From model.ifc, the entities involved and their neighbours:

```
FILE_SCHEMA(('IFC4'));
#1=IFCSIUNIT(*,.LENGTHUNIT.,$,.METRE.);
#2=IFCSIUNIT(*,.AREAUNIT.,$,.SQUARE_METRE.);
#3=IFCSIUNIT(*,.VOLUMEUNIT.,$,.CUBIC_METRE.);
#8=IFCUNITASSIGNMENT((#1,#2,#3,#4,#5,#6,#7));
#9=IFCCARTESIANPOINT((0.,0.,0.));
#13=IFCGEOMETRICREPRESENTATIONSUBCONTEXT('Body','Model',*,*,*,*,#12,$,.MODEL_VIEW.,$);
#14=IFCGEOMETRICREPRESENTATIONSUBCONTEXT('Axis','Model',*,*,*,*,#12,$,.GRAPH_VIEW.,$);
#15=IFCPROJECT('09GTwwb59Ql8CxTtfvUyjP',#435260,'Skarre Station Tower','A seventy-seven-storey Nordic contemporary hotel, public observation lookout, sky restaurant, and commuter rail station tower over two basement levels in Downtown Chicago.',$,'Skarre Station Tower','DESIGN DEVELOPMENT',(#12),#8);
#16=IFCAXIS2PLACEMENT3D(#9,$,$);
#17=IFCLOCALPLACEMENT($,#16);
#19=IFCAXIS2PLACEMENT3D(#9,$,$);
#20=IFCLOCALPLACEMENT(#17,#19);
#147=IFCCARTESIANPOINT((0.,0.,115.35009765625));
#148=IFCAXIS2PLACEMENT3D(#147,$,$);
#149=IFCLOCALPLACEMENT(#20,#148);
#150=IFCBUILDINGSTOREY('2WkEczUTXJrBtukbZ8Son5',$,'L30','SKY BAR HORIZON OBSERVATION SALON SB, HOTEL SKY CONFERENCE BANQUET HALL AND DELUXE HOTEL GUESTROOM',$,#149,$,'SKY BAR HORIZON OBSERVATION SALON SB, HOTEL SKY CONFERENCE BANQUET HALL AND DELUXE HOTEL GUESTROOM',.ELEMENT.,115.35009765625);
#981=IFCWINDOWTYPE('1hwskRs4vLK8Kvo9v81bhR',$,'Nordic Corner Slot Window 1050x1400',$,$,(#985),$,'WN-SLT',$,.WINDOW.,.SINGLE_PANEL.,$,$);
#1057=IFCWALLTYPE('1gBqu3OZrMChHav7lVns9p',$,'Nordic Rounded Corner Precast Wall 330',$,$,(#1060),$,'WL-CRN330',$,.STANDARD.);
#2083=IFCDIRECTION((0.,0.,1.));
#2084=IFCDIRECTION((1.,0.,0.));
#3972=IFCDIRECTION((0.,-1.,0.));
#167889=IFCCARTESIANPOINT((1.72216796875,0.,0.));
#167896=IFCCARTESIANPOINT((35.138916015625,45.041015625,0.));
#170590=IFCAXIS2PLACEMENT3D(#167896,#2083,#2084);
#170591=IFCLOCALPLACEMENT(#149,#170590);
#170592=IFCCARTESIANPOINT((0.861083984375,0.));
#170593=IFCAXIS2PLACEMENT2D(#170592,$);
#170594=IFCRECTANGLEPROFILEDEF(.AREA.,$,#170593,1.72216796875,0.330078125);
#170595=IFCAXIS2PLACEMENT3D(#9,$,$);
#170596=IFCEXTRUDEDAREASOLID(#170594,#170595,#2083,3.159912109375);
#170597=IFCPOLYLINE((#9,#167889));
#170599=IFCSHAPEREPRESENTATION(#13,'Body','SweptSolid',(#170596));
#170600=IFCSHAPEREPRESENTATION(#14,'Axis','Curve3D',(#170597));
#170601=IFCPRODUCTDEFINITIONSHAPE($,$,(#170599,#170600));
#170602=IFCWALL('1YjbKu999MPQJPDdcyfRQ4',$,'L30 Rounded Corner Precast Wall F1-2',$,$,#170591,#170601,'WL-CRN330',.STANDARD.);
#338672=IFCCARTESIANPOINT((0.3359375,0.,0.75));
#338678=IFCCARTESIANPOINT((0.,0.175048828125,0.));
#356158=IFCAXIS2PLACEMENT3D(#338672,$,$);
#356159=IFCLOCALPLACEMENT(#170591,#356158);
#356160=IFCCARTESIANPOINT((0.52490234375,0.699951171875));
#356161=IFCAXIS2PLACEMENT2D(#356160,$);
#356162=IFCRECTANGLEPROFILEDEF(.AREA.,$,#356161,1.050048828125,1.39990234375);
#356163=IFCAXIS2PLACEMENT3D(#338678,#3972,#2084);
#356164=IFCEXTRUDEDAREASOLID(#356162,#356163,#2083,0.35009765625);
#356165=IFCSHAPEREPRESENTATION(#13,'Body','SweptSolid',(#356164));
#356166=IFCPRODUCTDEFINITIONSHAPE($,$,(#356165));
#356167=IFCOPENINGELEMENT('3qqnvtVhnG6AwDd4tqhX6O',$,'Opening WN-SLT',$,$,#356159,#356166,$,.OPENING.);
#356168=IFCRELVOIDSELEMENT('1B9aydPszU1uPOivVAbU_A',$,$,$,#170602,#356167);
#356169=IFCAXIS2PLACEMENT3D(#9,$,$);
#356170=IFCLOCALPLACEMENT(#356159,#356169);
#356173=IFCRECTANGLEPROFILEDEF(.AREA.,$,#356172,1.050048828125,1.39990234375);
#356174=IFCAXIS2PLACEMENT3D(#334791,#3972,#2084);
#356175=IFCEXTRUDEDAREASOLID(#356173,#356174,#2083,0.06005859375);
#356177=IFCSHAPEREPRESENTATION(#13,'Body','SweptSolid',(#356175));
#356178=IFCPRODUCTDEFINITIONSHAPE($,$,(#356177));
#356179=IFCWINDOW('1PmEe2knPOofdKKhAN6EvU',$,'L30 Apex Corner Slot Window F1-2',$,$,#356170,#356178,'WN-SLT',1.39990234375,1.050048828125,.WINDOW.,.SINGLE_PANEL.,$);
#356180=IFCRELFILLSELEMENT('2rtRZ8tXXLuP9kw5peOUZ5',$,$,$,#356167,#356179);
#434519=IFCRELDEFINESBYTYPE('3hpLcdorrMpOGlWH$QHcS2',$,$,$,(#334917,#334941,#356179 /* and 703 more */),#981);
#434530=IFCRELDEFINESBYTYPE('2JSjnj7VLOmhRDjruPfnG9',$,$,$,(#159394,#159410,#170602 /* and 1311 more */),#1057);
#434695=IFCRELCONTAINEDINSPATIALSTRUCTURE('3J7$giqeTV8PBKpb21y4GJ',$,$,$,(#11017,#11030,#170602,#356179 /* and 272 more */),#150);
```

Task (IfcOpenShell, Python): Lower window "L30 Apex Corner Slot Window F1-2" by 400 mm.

```python
import numpy as np
import ifcopenshell
import ifcopenshell.api.geometry
import ifcopenshell.util.placement
import ifcopenshell.util.unit

model = ifcopenshell.open("model.ifc")
unit_scale = ifcopenshell.util.unit.calculate_unit_scale(model)

window = model.by_id(356179)
opening = window.FillsVoids[0].RelatingOpeningElement
dz = -0.4

shift = np.array([0.0, 0.0, dz])
# The window is placed relative to its opening, so it follows when the opening moves.
matrix = ifcopenshell.util.placement.get_local_placement(opening.ObjectPlacement)
matrix[:3, 3] += shift
ifcopenshell.api.geometry.edit_object_placement(
    model, product=opening, matrix=matrix, is_si=False, should_transform_children=True
)

print(f"moved by {dz * unit_scale:+.3f} m")

model.write("model_updated.ifc")
```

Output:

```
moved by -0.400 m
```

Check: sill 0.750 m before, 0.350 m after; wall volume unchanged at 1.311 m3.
